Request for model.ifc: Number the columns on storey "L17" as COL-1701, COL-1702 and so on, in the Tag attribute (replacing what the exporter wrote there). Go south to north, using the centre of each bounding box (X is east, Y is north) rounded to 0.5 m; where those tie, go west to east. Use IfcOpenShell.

First a look at what the model holds.

```python
import ifcopenshell
import ifcopenshell.util.element
import ifcopenshell.util.placement

model = ifcopenshell.open("model.ifc")
print(model.schema)
storey = next(s for s in model.by_type("IfcBuildingStorey") if s.Name == "L17")
columns = [e for e in ifcopenshell.util.element.get_decomposition(storey) if e.is_a("IfcColumn")]
for e in sorted(columns, key=lambda e: e.id()):
    origin = ifcopenshell.util.placement.get_local_placement(e.ObjectPlacement)[:3, 3]
    print(e.id(), e.Tag, e.Name, origin.round(2) + 0.0, sep=" | ")
```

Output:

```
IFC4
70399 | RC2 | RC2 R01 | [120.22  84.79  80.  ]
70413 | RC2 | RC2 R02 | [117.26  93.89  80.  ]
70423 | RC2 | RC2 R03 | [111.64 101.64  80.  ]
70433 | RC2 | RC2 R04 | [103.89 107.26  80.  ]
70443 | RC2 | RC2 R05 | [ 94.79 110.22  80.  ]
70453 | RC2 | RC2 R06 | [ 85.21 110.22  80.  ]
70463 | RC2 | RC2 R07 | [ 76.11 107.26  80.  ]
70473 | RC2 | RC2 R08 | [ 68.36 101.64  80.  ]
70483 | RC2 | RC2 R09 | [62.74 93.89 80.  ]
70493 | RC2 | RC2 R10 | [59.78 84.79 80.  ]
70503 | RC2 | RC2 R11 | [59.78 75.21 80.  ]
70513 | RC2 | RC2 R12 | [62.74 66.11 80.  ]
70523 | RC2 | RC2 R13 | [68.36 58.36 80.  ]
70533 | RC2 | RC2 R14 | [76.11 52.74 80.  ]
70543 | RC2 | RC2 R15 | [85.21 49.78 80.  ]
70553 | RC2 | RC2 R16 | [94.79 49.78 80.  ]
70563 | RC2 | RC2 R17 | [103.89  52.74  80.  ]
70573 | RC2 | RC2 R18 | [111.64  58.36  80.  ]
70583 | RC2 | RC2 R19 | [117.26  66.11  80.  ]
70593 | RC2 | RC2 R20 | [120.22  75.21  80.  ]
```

```python
import ifcopenshell
import ifcopenshell.geom
import ifcopenshell.util.element
import ifcopenshell.util.shape

model = ifcopenshell.open("model.ifc")
settings = ifcopenshell.geom.settings()
settings.set("use-world-coords", True)


def centre(element):
    shape = ifcopenshell.geom.create_shape(settings, element)
    return ifcopenshell.util.shape.get_bbox_centroid(shape.geometry)


storey = next(s for s in model.by_type("IfcBuildingStorey") if s.Name == "L17")
columns = [e for e in ifcopenshell.util.element.get_decomposition(storey) if e.is_a("IfcColumn")]

# Insertion points can sit at a corner or the storey origin, so sort by the geometry (in metres).
centres = {e: centre(e) for e in columns}
columns.sort(key=lambda e: (round(centres[e][1] / 0.5), centres[e][0]))

for i, e in enumerate(columns, start=1):
    number = f"COL-17{i:02d}"
    e.Tag = number
    print(e.id(), number)

model.write("model_rev.ifc")
```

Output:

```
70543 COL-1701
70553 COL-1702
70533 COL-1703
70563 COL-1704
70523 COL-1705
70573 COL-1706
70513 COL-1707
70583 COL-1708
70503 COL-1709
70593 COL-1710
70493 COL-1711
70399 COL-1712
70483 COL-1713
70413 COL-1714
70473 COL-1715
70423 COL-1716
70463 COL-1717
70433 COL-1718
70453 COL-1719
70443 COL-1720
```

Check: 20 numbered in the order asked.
